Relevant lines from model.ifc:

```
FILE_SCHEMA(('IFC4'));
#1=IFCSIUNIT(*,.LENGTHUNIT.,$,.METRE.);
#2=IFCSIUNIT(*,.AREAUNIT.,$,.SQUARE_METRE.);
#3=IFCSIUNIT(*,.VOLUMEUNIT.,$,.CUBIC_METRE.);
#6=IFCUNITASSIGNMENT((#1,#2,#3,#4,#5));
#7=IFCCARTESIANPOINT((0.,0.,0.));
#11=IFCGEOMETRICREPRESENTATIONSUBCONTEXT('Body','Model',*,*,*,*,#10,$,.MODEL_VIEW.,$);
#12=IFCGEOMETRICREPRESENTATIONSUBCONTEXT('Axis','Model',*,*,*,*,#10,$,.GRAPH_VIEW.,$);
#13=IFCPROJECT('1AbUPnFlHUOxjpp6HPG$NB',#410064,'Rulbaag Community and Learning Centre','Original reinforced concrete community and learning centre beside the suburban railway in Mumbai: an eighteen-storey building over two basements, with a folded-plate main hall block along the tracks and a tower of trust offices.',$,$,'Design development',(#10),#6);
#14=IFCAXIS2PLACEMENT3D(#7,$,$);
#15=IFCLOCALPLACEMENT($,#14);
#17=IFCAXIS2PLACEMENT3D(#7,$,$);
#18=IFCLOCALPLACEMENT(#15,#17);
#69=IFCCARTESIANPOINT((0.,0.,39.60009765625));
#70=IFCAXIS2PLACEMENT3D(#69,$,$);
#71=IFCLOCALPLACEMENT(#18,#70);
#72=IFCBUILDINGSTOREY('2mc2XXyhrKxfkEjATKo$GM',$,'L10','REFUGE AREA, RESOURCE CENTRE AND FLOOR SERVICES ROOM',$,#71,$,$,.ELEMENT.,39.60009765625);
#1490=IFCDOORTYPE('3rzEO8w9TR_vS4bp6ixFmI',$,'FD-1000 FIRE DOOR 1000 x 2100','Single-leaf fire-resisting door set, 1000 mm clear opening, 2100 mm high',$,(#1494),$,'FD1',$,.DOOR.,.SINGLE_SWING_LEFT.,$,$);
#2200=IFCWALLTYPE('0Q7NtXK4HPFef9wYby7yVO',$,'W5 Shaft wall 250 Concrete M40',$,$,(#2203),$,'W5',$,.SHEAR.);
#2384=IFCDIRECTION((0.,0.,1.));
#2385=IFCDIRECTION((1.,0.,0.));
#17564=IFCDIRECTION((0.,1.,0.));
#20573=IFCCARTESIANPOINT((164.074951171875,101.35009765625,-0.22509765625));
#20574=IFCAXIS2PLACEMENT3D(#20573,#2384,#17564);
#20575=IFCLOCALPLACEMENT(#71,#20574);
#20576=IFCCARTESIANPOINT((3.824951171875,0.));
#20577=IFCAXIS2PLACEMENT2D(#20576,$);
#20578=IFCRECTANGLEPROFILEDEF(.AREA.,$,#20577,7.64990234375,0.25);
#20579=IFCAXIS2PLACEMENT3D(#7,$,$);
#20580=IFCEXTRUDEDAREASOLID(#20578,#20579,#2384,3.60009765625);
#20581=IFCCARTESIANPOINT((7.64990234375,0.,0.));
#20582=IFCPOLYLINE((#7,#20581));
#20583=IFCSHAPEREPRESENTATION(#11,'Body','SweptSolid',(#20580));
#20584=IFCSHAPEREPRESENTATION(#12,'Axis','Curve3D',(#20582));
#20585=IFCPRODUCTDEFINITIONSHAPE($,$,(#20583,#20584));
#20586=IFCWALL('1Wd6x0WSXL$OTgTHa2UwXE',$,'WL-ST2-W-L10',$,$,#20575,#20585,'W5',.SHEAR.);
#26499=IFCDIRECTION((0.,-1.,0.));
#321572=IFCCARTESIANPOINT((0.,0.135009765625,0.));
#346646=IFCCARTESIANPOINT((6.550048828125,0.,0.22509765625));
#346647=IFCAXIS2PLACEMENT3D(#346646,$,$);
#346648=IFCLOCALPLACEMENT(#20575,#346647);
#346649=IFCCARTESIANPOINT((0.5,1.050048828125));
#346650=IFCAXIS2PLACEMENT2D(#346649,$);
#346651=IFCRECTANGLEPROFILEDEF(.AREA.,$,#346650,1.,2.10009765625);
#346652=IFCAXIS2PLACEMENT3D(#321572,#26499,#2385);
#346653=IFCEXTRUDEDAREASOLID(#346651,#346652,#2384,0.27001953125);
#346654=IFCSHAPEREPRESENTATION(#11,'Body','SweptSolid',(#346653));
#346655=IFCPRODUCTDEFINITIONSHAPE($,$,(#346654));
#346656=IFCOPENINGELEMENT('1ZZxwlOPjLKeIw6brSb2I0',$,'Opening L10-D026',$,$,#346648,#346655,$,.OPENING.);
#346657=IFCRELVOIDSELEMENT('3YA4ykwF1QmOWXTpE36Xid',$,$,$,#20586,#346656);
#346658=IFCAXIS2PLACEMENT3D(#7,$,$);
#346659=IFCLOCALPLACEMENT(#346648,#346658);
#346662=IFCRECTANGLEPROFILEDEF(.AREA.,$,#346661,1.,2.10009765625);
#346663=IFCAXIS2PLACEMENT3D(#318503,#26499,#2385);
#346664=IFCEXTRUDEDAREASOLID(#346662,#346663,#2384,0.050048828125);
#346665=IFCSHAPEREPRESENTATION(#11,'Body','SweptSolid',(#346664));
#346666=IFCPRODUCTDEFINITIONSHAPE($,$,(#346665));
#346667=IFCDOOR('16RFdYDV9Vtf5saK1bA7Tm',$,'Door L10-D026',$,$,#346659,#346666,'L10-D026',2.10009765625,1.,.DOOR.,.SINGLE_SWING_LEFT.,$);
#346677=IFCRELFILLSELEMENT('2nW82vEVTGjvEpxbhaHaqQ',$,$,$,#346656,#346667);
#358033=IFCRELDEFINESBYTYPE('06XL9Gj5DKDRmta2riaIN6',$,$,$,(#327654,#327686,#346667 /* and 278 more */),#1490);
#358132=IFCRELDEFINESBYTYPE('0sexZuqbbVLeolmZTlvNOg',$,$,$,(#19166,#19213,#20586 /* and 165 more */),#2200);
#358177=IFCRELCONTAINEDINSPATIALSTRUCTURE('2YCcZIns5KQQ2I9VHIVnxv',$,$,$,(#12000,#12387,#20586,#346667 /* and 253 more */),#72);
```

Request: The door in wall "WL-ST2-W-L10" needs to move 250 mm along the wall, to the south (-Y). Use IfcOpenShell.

```python
import ifcopenshell
import ifcopenshell.api.geometry
import ifcopenshell.util.placement

model = ifcopenshell.open("model.ifc")

door = model.by_guid("16RFdYDV9Vtf5saK1bA7Tm")
opening = door.FillsVoids[0].RelatingOpeningElement
wall = opening.VoidsElements[0].RelatingBuildingElement

wall_matrix = ifcopenshell.util.placement.get_local_placement(wall.ObjectPlacement)
shift = wall_matrix[:3, 0] * -0.25
before = ifcopenshell.util.placement.get_local_placement(door.ObjectPlacement)[:3, 3].copy()

# The door is placed relative to its opening, so it follows when the opening moves.
matrix = ifcopenshell.util.placement.get_local_placement(opening.ObjectPlacement)
matrix[:3, 3] += shift
ifcopenshell.api.geometry.edit_object_placement(
    model, product=opening, matrix=matrix, is_si=False, should_transform_children=True
)

after = ifcopenshell.util.placement.get_local_placement(door.ObjectPlacement)[:3, 3]
print("door moved by", (after - before).round(3) + 0.0)

model.write("model-out.ifc")
```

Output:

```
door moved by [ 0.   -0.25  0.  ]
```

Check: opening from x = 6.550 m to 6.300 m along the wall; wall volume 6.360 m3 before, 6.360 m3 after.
